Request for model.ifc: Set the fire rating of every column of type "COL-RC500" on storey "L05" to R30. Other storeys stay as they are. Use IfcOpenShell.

First a look at what the model holds.

```python
import ifcopenshell
import ifcopenshell.util.element

model = ifcopenshell.open("model.ifc")
print(model.schema)
storey = next(s for s in model.by_type("IfcBuildingStorey") if s.Name == "L05")
columns = [e for e in ifcopenshell.util.element.get_decomposition(storey) if e.is_a("IfcColumn")]
seen = {}
for e in columns:
    element_type = ifcopenshell.util.element.get_type(e)
    key = (element_type.Name if element_type != e and element_type else None, ifcopenshell.util.element.get_pset(e, "Pset_ColumnCommon", "FireRating"))
    seen[key] = seen.get(key, 0) + 1
for (name, value), count in sorted(seen.items(), key=str):
    print(count, "x", name, "|", value)
```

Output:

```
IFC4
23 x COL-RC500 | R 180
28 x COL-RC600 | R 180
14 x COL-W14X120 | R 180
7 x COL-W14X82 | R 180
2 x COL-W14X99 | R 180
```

```python
import ifcopenshell
import ifcopenshell.api.pset
import ifcopenshell.util.element

model = ifcopenshell.open("model.ifc")

storey = next(s for s in model.by_type("IfcBuildingStorey") if s.Name == "L05")
columns = [e for e in ifcopenshell.util.element.get_decomposition(storey) if e.is_a("IfcColumn")]

count = 0
for e in columns:
    element_type = ifcopenshell.util.element.get_type(e)
    if element_type in (None, e) or element_type.Name != "COL-RC500":
        continue
    # add_pset returns the element's existing set when there is one.
    pset = ifcopenshell.api.pset.add_pset(model, product=e, name="Pset_ColumnCommon")
    ifcopenshell.api.pset.edit_pset(model, pset=pset, properties={"FireRating": "R30"})
    count += 1

print(count, "columns updated")

model.write("model_edited.ifc")
```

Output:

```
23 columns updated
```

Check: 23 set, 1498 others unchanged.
